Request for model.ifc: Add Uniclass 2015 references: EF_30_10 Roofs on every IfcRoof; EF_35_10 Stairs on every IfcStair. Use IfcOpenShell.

First a look at what the model holds.

```python
import ifcopenshell

model = ifcopenshell.open("model.ifc")
print(model.schema)
print("classifications:", [c.Name for c in model.by_type("IfcClassification")])
for ifc_class in ("IfcDoor", "IfcRoof", "IfcStair", "IfcWall", "IfcWindow"):
    print(ifc_class, len(model.by_type(ifc_class)))
```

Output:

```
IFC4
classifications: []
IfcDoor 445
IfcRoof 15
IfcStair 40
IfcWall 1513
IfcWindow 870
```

```python
import ifcopenshell
import ifcopenshell.api.classification

model = ifcopenshell.open("model.ifc")

system = ifcopenshell.api.classification.add_classification(model, classification="Uniclass 2015")

codes = {
    "IfcRoof": ("EF_30_10", "Roofs"),
    "IfcStair": ("EF_35_10", "Stairs"),
}
for ifc_class, (code, name) in codes.items():
    products = model.by_type(ifc_class)
    ifcopenshell.api.classification.add_reference(
        model, products=products, classification=system, identification=code, name=name
    )
    print(code, len(products))

model.write("model_updated.ifc")
```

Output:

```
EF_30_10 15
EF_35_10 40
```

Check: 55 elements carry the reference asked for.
